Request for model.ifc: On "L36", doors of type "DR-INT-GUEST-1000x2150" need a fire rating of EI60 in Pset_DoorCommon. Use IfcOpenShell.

First a look at what the model holds.

```python
import ifcopenshell
import ifcopenshell.util.element

model = ifcopenshell.open("model.ifc")
print(model.schema)
storey = next(s for s in model.by_type("IfcBuildingStorey") if s.Name == "L36")
doors = [e for e in ifcopenshell.util.element.get_decomposition(storey) if e.is_a("IfcDoor")]
seen = {}
for e in doors:
    element_type = ifcopenshell.util.element.get_type(e)
    key = (element_type.Name if element_type != e and element_type else None, ifcopenshell.util.element.get_pset(e, "Pset_DoorCommon", "FireRating"))
    seen[key] = seen.get(key, 0) + 1
for (name, value), count in sorted(seen.items(), key=str):
    print(count, "x", name, "|", value)
```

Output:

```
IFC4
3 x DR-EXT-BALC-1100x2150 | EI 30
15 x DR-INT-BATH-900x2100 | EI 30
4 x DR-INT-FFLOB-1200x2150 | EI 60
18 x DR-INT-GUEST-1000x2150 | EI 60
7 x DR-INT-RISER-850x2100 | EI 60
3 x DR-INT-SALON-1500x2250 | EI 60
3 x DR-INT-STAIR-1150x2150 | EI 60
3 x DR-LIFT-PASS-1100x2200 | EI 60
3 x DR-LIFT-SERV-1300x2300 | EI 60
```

```python
import ifcopenshell
import ifcopenshell.api.pset
import ifcopenshell.util.element

model = ifcopenshell.open("model.ifc")

storey = next(s for s in model.by_type("IfcBuildingStorey") if s.Name == "L36")
doors = [e for e in ifcopenshell.util.element.get_decomposition(storey) if e.is_a("IfcDoor")]

count = 0
for e in doors:
    element_type = ifcopenshell.util.element.get_type(e)
    if element_type in (None, e) or element_type.Name != "DR-INT-GUEST-1000x2150":
        continue
    # add_pset returns the element's existing set when there is one.
    pset = ifcopenshell.api.pset.add_pset(model, product=e, name="Pset_DoorCommon")
    ifcopenshell.api.pset.edit_pset(model, pset=pset, properties={"FireRating": "EI60"})
    count += 1

print(count, "doors updated")

model.write("model_edited.ifc")
```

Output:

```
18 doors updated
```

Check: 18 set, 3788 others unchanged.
